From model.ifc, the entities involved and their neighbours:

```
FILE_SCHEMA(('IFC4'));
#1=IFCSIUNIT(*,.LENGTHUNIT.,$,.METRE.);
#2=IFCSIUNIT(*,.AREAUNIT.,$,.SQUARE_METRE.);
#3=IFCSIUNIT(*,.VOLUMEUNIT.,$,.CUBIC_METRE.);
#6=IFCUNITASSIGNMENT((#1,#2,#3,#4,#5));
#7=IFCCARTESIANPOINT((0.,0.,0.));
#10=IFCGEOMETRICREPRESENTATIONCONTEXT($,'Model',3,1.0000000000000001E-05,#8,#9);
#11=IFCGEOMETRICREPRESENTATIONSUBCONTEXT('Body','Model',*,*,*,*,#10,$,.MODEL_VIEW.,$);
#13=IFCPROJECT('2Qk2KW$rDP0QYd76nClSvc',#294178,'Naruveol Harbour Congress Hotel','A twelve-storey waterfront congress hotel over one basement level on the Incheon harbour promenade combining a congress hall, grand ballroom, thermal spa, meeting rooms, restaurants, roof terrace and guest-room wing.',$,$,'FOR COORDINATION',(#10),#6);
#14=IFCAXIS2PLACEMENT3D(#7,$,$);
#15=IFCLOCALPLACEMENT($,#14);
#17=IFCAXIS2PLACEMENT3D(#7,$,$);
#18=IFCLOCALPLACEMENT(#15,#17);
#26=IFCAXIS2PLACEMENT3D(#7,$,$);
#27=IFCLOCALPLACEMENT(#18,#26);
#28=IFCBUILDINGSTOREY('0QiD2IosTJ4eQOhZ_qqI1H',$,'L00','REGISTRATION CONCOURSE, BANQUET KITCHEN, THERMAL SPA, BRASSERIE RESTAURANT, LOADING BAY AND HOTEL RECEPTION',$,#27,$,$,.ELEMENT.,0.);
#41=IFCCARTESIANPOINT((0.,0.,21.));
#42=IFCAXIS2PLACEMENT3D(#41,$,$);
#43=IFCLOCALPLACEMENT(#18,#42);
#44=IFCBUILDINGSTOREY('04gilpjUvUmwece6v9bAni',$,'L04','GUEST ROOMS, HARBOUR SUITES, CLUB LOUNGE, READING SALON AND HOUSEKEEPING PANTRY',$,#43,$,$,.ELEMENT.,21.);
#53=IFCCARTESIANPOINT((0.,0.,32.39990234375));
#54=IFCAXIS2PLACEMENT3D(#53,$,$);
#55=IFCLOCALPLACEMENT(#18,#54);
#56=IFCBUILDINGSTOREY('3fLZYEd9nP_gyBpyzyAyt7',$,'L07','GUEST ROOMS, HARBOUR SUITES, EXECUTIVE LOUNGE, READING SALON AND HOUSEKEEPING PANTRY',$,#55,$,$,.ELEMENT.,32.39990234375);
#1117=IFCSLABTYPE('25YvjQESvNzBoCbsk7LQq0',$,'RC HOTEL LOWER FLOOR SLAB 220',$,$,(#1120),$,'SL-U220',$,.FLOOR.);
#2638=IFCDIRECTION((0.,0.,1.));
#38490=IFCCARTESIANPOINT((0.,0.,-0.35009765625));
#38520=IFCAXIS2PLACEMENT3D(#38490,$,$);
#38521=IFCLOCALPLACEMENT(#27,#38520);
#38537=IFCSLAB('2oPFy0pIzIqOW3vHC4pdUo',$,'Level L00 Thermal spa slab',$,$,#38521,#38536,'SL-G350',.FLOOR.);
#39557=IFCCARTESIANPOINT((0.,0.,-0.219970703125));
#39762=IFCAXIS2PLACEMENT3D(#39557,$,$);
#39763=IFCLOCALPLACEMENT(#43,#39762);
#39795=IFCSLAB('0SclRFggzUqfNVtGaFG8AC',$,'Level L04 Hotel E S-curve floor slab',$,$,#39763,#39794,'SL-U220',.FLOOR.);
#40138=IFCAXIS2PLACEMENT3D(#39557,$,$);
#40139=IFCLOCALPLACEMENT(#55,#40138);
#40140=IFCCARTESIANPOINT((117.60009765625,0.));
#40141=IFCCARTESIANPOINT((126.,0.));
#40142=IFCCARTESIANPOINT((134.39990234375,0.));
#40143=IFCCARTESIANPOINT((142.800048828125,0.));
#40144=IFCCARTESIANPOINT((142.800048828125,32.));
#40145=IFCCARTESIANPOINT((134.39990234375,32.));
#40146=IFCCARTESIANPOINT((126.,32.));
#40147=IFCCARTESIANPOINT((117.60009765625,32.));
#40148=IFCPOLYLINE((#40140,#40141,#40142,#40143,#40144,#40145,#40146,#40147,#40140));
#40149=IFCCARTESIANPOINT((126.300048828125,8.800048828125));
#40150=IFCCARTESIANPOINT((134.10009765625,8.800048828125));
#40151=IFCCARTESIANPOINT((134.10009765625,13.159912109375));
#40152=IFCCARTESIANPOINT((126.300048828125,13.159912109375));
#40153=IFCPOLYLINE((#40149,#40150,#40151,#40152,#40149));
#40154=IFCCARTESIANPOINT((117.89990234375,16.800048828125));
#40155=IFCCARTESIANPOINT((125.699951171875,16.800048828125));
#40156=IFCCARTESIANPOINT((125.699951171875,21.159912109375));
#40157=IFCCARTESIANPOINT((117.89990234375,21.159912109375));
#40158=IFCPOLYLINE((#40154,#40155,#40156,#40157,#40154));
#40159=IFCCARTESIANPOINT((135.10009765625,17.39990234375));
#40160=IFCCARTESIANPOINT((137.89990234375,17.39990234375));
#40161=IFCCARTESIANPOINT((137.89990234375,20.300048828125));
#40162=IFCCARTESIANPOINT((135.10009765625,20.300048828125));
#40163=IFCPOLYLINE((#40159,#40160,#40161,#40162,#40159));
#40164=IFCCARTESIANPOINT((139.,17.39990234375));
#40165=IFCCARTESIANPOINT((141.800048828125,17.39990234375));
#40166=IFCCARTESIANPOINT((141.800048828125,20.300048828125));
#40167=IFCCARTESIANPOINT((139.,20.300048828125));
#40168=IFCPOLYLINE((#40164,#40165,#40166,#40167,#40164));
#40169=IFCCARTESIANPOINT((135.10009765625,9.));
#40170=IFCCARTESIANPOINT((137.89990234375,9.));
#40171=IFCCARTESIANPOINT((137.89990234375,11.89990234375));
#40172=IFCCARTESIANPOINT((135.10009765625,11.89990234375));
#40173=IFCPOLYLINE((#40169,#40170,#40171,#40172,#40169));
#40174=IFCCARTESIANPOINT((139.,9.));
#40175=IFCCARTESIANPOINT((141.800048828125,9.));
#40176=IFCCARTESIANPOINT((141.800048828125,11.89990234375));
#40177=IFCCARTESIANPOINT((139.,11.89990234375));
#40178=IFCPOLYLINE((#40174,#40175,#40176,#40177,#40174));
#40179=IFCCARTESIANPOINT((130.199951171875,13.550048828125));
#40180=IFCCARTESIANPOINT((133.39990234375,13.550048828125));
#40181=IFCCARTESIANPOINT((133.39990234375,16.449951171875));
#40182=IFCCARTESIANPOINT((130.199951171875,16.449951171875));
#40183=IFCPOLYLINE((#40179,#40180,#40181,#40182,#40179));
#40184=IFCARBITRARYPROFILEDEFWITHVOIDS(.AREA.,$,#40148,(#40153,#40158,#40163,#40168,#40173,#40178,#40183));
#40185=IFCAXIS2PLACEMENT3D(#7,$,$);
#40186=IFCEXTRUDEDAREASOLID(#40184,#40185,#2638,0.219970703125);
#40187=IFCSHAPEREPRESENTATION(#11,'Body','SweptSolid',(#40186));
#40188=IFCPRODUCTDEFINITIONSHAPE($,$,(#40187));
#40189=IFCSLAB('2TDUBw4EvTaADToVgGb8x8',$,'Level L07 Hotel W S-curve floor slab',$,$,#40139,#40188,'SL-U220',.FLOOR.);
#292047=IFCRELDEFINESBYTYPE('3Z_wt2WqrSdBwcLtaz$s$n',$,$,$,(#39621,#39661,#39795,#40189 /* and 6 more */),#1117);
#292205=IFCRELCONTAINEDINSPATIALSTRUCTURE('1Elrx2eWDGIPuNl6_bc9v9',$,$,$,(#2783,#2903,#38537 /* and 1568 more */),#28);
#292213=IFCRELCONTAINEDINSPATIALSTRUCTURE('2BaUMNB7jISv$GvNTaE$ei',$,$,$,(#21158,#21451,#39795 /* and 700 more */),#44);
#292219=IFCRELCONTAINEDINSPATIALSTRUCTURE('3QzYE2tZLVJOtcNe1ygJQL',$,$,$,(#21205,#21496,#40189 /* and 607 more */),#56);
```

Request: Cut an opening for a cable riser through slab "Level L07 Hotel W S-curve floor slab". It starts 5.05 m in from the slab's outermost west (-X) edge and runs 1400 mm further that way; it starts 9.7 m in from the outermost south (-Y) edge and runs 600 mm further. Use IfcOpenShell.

```python
import numpy as np
import ifcopenshell
import ifcopenshell.api.feature
import ifcopenshell.api.geometry
import ifcopenshell.api.root
import ifcopenshell.geom
import ifcopenshell.util.placement
import ifcopenshell.util.representation
import ifcopenshell.util.shape
import ifcopenshell.util.unit

model = ifcopenshell.open("model.ifc")
unit_scale = ifcopenshell.util.unit.calculate_unit_scale(model)
settings = ifcopenshell.geom.settings()


def volume(element):
    """Net volume in cubic metres, openings subtracted."""
    shape = ifcopenshell.geom.create_shape(settings, element)
    return ifcopenshell.util.shape.get_volume(shape.geometry)


slab = model.by_id(40189)
before = volume(slab)

# Extent in the slab's own axes, in metres. The edges named are its -X and -Y sides.
slab_shape = ifcopenshell.geom.create_shape(settings, slab)
vertices = ifcopenshell.util.shape.get_vertices(slab_shape.geometry)
x_min, y_min, bottom = vertices.min(axis=0)
top = vertices[:, 2].max()

opening = ifcopenshell.api.root.create_entity(model, ifc_class="IfcOpeningElement", name="Cable riser opening", predefined_type="OPENING")
context = ifcopenshell.util.representation.get_context(model, "Model", "Body", "MODEL_VIEW")
width, depth = 1.4, 0.6
outline = [(0.0, 0.0), (width, 0.0), (width, depth), (0.0, depth), (0.0, 0.0)]
# Overshoot both faces by 50 mm so the cut is clean.
shape = ifcopenshell.api.geometry.add_slab_representation(
    model, context=context, depth=top - bottom + 0.1, polyline=outline
)
ifcopenshell.api.geometry.assign_representation(model, product=opening, representation=shape)

matrix = ifcopenshell.util.placement.get_local_placement(slab.ObjectPlacement)
matrix[:, 3] = matrix @ np.append(np.array([x_min + 5.05, y_min + 9.7, bottom - 0.05]) / unit_scale, 1.0)
ifcopenshell.api.geometry.edit_object_placement(model, product=opening, matrix=matrix, is_si=False)
ifcopenshell.api.feature.add_feature(model, feature=opening, element=slab)

after = volume(slab)

print(f"slab volume {before:.3f} -> {after:.3f} m3")

model.write("model_v2.ifc")
```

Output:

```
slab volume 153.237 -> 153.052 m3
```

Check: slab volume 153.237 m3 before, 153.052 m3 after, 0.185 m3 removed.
